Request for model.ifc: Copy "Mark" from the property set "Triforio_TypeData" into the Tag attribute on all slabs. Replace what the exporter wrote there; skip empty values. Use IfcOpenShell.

First a look at what the model holds.

```python
import ifcopenshell
import ifcopenshell.util.element

model = ifcopenshell.open("model.ifc")
print(model.schema)
slabs = model.by_type("IfcSlab")
print(len(slabs), "slabs")
for e in slabs[:8]:
    source = ifcopenshell.util.element.get_pset(e, "Triforio_TypeData", "Mark")
    target = e.Tag
    print(e.id(), repr(source), repr(target), sep=" | ")
```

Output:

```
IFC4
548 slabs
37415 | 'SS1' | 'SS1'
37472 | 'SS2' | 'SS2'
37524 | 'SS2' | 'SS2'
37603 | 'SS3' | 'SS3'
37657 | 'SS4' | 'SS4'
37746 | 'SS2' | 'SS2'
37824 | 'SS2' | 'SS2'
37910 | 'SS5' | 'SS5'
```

```python
import ifcopenshell
import ifcopenshell.util.element

model = ifcopenshell.open("model.ifc")

count = 0
for e in model.by_type("IfcSlab"):
    value = ifcopenshell.util.element.get_pset(e, "Triforio_TypeData", "Mark")
    current = e.Tag
    if not value or not value.strip() or current == value:
        continue
    e.Tag = value
    count += 1

print(count, "slabs updated")

model.write("model_edited.ifc")
```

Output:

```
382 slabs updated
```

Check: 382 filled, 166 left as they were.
